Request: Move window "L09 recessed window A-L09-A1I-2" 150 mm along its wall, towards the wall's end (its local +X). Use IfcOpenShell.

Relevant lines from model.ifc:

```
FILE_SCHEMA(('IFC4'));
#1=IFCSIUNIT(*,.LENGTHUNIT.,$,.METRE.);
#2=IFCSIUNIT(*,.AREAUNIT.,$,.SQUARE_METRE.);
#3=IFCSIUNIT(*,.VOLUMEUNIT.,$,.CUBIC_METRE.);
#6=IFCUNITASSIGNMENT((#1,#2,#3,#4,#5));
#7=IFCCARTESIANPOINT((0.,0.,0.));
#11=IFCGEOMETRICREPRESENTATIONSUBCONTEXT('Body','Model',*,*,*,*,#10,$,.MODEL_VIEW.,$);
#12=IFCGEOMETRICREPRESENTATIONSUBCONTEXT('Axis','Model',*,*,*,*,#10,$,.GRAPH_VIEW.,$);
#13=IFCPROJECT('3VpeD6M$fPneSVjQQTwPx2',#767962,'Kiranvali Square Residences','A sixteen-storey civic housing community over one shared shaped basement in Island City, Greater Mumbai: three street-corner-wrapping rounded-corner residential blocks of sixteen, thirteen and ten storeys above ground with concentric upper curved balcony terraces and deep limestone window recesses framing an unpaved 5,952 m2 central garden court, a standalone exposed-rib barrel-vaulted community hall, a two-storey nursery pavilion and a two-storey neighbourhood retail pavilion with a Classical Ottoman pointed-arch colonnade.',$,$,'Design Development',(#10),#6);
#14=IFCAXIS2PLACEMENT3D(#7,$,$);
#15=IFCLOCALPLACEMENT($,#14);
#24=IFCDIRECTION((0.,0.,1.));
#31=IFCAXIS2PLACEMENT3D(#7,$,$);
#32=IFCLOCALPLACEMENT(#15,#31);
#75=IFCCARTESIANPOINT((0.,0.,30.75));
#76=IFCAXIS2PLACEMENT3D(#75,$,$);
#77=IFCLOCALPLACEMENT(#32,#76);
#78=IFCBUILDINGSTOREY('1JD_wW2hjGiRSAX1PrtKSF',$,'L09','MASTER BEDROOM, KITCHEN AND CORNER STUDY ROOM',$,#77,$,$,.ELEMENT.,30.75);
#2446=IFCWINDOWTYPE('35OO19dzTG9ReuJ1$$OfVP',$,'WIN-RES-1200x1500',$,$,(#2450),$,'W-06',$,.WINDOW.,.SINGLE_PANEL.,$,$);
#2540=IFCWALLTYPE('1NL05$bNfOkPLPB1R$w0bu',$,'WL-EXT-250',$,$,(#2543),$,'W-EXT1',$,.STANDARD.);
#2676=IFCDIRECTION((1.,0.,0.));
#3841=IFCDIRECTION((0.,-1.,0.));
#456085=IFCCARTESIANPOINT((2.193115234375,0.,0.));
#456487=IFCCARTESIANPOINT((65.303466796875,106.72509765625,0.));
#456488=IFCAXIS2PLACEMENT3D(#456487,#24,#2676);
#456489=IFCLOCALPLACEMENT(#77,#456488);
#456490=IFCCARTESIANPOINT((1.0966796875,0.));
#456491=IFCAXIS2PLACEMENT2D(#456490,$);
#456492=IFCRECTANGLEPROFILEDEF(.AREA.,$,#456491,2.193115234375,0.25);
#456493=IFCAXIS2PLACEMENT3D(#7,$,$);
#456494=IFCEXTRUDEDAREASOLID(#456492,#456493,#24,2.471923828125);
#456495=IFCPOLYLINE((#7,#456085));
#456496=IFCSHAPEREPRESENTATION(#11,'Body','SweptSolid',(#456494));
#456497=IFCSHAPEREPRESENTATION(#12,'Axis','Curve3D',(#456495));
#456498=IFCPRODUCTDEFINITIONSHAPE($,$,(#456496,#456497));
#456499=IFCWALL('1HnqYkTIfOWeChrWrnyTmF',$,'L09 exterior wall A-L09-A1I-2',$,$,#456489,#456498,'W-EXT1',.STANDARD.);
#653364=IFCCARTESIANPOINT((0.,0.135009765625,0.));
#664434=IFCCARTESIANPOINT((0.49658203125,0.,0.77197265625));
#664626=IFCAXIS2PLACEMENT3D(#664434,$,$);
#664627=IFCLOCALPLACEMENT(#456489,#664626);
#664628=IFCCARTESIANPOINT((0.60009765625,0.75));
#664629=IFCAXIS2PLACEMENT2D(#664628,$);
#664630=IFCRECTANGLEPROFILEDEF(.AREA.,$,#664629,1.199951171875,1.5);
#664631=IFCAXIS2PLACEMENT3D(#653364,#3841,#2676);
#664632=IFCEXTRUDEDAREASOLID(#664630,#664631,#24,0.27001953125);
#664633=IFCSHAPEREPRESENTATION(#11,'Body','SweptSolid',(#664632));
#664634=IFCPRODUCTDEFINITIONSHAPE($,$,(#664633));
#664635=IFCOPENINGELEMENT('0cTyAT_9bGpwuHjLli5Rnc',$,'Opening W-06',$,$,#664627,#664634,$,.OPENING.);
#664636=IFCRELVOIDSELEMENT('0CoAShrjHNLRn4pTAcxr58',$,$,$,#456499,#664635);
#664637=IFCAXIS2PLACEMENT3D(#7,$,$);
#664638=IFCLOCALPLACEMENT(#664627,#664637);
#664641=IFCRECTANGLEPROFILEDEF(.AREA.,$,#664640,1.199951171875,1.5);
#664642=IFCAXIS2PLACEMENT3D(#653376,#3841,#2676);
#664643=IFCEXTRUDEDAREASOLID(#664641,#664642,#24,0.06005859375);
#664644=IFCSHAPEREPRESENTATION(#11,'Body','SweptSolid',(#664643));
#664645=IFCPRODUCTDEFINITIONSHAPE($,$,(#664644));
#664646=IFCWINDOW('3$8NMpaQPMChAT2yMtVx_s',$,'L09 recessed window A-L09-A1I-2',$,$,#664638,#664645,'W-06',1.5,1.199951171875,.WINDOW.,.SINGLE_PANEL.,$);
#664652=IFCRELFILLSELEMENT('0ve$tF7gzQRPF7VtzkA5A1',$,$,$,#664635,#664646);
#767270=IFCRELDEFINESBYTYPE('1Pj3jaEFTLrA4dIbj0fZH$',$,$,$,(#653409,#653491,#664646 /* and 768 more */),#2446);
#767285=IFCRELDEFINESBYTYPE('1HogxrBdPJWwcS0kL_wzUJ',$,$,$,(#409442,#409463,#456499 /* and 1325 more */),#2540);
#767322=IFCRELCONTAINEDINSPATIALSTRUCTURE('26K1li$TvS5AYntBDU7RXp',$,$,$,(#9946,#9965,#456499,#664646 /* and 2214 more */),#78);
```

```python
import ifcopenshell
import ifcopenshell.api.geometry
import ifcopenshell.util.placement

model = ifcopenshell.open("model.ifc")

window = model.by_id(664646)
opening = window.FillsVoids[0].RelatingOpeningElement
wall = opening.VoidsElements[0].RelatingBuildingElement

wall_matrix = ifcopenshell.util.placement.get_local_placement(wall.ObjectPlacement)
shift = wall_matrix[:3, 0] * 0.15
before = ifcopenshell.util.placement.get_local_placement(window.ObjectPlacement)[:3, 3].copy()

# The window is placed relative to its opening, so it follows when the opening moves.
matrix = ifcopenshell.util.placement.get_local_placement(opening.ObjectPlacement)
matrix[:3, 3] += shift
ifcopenshell.api.geometry.edit_object_placement(
    model, product=opening, matrix=matrix, is_si=False, should_transform_children=True
)

after = ifcopenshell.util.placement.get_local_placement(window.ObjectPlacement)[:3, 3]
print("window moved by", (after - before).round(3) + 0.0)

model.write("model_updated.ifc")
```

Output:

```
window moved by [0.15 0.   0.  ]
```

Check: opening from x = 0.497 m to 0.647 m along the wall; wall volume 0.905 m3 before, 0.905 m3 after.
